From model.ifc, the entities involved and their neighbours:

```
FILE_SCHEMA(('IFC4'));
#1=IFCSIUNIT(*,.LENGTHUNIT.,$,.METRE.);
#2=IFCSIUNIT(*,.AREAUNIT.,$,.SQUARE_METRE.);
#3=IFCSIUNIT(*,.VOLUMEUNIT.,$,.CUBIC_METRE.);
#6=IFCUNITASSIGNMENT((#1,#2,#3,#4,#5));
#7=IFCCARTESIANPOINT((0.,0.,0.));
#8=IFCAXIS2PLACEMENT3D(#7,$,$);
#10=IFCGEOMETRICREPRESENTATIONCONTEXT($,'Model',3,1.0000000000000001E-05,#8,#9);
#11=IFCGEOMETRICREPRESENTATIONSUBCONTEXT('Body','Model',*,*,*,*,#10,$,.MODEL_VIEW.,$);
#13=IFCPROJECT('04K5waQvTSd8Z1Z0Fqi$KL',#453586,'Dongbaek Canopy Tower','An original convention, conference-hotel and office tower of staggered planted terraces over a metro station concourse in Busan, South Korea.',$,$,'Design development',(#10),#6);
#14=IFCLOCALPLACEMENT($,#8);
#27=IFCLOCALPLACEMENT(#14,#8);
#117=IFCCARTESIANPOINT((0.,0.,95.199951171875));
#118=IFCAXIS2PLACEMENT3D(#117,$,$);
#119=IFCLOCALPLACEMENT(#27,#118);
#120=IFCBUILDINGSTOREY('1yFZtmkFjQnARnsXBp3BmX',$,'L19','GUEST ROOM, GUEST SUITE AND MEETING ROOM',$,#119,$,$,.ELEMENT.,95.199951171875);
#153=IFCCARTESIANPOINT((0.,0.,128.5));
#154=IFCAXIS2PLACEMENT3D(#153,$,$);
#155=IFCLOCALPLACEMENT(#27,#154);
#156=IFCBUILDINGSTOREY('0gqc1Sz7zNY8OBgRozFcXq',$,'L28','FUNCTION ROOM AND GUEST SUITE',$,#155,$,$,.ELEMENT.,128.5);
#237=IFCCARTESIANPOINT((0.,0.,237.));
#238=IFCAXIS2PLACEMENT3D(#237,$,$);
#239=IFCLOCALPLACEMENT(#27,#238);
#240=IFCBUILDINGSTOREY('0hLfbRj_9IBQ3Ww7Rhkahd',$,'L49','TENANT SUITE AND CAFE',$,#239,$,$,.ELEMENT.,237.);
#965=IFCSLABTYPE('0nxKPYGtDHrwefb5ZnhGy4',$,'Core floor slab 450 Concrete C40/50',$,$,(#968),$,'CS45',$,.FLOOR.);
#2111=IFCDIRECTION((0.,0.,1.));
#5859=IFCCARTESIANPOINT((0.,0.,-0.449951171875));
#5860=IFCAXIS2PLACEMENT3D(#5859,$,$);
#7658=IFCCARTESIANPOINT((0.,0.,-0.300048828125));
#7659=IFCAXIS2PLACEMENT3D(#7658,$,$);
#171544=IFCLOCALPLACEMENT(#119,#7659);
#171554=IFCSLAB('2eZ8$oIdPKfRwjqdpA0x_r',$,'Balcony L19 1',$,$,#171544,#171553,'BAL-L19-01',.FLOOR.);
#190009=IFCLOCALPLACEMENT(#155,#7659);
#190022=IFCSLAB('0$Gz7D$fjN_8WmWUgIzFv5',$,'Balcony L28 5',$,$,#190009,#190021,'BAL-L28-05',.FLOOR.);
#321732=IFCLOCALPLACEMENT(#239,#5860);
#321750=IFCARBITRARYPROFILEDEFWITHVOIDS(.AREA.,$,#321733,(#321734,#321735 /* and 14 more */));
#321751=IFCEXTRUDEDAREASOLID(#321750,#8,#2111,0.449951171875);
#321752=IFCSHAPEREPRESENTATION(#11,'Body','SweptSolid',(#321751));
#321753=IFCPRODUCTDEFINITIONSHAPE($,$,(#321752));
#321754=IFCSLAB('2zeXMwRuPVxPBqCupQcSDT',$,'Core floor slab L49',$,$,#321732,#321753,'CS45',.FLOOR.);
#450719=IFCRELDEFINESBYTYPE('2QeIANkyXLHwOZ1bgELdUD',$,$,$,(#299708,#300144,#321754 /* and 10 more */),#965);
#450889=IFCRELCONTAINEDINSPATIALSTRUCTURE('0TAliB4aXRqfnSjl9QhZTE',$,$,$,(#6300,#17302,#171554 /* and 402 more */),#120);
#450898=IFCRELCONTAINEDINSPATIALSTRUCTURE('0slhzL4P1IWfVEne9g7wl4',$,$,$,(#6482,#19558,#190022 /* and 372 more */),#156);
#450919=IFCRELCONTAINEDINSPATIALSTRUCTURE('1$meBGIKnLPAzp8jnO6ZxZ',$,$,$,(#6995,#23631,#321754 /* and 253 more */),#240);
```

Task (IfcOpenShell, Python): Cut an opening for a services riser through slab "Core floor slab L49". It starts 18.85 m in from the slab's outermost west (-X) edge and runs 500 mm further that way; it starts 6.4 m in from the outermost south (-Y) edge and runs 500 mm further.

```python
import numpy as np
import ifcopenshell
import ifcopenshell.api.feature
import ifcopenshell.api.geometry
import ifcopenshell.api.root
import ifcopenshell.geom
import ifcopenshell.util.placement
import ifcopenshell.util.representation
import ifcopenshell.util.shape
import ifcopenshell.util.unit

model = ifcopenshell.open("model.ifc")
unit_scale = ifcopenshell.util.unit.calculate_unit_scale(model)
settings = ifcopenshell.geom.settings()


def volume(element):
    """Net volume in cubic metres, openings subtracted."""
    shape = ifcopenshell.geom.create_shape(settings, element)
    return ifcopenshell.util.shape.get_volume(shape.geometry)


slab = model.by_id(321754)
before = volume(slab)

# Extent in the slab's own axes, in metres. The edges named are its -X and -Y sides.
slab_shape = ifcopenshell.geom.create_shape(settings, slab)
vertices = ifcopenshell.util.shape.get_vertices(slab_shape.geometry)
x_min, y_min, bottom = vertices.min(axis=0)
top = vertices[:, 2].max()

opening = ifcopenshell.api.root.create_entity(model, ifc_class="IfcOpeningElement", name="Services riser opening", predefined_type="OPENING")
context = ifcopenshell.util.representation.get_context(model, "Model", "Body", "MODEL_VIEW")
width, depth = 0.5, 0.5
outline = [(0.0, 0.0), (width, 0.0), (width, depth), (0.0, depth), (0.0, 0.0)]
# Overshoot both faces by 50 mm so the cut is clean.
shape = ifcopenshell.api.geometry.add_slab_representation(
    model, context=context, depth=top - bottom + 0.1, polyline=outline
)
ifcopenshell.api.geometry.assign_representation(model, product=opening, representation=shape)

matrix = ifcopenshell.util.placement.get_local_placement(slab.ObjectPlacement)
matrix[:, 3] = matrix @ np.append(np.array([x_min + 18.85, y_min + 6.4, bottom - 0.05]) / unit_scale, 1.0)
ifcopenshell.api.geometry.edit_object_placement(model, product=opening, matrix=matrix, is_si=False)
ifcopenshell.api.feature.add_feature(model, feature=opening, element=slab)

after = volume(slab)

print(f"slab volume {before:.3f} -> {after:.3f} m3")

model.write("model_rev.ifc")
```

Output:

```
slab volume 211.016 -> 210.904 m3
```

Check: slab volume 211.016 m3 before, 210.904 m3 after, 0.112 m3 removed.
